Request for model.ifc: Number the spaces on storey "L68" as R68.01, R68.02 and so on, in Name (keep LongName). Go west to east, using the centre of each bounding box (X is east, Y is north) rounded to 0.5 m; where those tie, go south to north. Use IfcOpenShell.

First a look at what the model holds.

```python
import ifcopenshell
import ifcopenshell.util.element
import ifcopenshell.util.placement

model = ifcopenshell.open("model.ifc")
print(model.schema)
storey = next(s for s in model.by_type("IfcBuildingStorey") if s.Name == "L68")
spaces = [e for e in ifcopenshell.util.element.get_decomposition(storey) if e.is_a("IfcSpace")]
for e in sorted(spaces, key=lambda e: e.id()):
    origin = ifcopenshell.util.placement.get_local_placement(e.ObjectPlacement)[:3, 3]
    print(e.id(), e.Name, e.LongName, origin.round(2) + 0.0, sep=" | ")
```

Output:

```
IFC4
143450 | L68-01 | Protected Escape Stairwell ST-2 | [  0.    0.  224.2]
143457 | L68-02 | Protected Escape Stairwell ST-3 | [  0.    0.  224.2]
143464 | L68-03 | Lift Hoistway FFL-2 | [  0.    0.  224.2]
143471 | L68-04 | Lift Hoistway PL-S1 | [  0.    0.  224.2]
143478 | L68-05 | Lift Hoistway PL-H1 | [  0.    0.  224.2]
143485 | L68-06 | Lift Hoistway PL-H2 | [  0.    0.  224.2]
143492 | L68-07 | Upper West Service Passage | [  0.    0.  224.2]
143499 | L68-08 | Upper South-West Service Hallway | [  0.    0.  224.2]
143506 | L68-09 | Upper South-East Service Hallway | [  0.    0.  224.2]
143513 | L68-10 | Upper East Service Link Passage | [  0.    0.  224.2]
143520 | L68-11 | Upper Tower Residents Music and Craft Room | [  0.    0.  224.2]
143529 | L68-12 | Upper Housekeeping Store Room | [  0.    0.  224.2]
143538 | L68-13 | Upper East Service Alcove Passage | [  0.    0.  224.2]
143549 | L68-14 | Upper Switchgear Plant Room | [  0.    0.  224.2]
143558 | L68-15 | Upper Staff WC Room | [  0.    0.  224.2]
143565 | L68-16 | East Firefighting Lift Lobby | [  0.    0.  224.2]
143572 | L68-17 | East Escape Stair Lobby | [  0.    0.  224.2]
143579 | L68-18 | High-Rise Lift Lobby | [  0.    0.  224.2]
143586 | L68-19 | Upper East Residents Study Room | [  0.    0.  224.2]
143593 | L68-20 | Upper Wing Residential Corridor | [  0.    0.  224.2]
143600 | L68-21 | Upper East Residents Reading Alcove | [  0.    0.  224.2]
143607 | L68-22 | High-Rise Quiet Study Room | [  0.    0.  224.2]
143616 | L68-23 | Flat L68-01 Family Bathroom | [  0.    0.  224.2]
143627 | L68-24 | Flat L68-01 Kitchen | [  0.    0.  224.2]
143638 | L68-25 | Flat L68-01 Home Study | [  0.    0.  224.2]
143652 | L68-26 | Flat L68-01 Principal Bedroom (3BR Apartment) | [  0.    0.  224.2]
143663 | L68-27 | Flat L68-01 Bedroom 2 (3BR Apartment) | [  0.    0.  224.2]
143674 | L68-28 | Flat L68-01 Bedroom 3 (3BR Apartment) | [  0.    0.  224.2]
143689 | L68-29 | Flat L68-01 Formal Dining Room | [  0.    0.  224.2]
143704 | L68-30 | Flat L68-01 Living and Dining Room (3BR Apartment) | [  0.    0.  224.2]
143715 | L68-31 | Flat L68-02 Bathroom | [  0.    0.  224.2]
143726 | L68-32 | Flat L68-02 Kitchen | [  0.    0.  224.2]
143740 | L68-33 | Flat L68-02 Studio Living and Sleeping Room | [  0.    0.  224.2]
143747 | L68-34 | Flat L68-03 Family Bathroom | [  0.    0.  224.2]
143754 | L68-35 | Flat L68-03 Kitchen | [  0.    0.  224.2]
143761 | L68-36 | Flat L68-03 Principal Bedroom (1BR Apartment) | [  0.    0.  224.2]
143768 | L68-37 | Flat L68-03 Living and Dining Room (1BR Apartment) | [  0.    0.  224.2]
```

```python
import ifcopenshell
import ifcopenshell.geom
import ifcopenshell.util.element
import ifcopenshell.util.shape

model = ifcopenshell.open("model.ifc")
settings = ifcopenshell.geom.settings()
settings.set("use-world-coords", True)


def centre(element):
    shape = ifcopenshell.geom.create_shape(settings, element)
    return ifcopenshell.util.shape.get_bbox_centroid(shape.geometry)


storey = next(s for s in model.by_type("IfcBuildingStorey") if s.Name == "L68")
spaces = [e for e in ifcopenshell.util.element.get_decomposition(storey) if e.is_a("IfcSpace")]

# Insertion points can sit at a corner or the storey origin, so sort by the geometry (in metres).
centres = {e: centre(e) for e in spaces}
spaces.sort(key=lambda e: (round(centres[e][0] / 0.5), centres[e][1]))

for i, e in enumerate(spaces, start=1):
    number = f"R68.{i:02d}"
    e.Name = number
    print(e.id(), number)

model.write("model_updated.ifc")
```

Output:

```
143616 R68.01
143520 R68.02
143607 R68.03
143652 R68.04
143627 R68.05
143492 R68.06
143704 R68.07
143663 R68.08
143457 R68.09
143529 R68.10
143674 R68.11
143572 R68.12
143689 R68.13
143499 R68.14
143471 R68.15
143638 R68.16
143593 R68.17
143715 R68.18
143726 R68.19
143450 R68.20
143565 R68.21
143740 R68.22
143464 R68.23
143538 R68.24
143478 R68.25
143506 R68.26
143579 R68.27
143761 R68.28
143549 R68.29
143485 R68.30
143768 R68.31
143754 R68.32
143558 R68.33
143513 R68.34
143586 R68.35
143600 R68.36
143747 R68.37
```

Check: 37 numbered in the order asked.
